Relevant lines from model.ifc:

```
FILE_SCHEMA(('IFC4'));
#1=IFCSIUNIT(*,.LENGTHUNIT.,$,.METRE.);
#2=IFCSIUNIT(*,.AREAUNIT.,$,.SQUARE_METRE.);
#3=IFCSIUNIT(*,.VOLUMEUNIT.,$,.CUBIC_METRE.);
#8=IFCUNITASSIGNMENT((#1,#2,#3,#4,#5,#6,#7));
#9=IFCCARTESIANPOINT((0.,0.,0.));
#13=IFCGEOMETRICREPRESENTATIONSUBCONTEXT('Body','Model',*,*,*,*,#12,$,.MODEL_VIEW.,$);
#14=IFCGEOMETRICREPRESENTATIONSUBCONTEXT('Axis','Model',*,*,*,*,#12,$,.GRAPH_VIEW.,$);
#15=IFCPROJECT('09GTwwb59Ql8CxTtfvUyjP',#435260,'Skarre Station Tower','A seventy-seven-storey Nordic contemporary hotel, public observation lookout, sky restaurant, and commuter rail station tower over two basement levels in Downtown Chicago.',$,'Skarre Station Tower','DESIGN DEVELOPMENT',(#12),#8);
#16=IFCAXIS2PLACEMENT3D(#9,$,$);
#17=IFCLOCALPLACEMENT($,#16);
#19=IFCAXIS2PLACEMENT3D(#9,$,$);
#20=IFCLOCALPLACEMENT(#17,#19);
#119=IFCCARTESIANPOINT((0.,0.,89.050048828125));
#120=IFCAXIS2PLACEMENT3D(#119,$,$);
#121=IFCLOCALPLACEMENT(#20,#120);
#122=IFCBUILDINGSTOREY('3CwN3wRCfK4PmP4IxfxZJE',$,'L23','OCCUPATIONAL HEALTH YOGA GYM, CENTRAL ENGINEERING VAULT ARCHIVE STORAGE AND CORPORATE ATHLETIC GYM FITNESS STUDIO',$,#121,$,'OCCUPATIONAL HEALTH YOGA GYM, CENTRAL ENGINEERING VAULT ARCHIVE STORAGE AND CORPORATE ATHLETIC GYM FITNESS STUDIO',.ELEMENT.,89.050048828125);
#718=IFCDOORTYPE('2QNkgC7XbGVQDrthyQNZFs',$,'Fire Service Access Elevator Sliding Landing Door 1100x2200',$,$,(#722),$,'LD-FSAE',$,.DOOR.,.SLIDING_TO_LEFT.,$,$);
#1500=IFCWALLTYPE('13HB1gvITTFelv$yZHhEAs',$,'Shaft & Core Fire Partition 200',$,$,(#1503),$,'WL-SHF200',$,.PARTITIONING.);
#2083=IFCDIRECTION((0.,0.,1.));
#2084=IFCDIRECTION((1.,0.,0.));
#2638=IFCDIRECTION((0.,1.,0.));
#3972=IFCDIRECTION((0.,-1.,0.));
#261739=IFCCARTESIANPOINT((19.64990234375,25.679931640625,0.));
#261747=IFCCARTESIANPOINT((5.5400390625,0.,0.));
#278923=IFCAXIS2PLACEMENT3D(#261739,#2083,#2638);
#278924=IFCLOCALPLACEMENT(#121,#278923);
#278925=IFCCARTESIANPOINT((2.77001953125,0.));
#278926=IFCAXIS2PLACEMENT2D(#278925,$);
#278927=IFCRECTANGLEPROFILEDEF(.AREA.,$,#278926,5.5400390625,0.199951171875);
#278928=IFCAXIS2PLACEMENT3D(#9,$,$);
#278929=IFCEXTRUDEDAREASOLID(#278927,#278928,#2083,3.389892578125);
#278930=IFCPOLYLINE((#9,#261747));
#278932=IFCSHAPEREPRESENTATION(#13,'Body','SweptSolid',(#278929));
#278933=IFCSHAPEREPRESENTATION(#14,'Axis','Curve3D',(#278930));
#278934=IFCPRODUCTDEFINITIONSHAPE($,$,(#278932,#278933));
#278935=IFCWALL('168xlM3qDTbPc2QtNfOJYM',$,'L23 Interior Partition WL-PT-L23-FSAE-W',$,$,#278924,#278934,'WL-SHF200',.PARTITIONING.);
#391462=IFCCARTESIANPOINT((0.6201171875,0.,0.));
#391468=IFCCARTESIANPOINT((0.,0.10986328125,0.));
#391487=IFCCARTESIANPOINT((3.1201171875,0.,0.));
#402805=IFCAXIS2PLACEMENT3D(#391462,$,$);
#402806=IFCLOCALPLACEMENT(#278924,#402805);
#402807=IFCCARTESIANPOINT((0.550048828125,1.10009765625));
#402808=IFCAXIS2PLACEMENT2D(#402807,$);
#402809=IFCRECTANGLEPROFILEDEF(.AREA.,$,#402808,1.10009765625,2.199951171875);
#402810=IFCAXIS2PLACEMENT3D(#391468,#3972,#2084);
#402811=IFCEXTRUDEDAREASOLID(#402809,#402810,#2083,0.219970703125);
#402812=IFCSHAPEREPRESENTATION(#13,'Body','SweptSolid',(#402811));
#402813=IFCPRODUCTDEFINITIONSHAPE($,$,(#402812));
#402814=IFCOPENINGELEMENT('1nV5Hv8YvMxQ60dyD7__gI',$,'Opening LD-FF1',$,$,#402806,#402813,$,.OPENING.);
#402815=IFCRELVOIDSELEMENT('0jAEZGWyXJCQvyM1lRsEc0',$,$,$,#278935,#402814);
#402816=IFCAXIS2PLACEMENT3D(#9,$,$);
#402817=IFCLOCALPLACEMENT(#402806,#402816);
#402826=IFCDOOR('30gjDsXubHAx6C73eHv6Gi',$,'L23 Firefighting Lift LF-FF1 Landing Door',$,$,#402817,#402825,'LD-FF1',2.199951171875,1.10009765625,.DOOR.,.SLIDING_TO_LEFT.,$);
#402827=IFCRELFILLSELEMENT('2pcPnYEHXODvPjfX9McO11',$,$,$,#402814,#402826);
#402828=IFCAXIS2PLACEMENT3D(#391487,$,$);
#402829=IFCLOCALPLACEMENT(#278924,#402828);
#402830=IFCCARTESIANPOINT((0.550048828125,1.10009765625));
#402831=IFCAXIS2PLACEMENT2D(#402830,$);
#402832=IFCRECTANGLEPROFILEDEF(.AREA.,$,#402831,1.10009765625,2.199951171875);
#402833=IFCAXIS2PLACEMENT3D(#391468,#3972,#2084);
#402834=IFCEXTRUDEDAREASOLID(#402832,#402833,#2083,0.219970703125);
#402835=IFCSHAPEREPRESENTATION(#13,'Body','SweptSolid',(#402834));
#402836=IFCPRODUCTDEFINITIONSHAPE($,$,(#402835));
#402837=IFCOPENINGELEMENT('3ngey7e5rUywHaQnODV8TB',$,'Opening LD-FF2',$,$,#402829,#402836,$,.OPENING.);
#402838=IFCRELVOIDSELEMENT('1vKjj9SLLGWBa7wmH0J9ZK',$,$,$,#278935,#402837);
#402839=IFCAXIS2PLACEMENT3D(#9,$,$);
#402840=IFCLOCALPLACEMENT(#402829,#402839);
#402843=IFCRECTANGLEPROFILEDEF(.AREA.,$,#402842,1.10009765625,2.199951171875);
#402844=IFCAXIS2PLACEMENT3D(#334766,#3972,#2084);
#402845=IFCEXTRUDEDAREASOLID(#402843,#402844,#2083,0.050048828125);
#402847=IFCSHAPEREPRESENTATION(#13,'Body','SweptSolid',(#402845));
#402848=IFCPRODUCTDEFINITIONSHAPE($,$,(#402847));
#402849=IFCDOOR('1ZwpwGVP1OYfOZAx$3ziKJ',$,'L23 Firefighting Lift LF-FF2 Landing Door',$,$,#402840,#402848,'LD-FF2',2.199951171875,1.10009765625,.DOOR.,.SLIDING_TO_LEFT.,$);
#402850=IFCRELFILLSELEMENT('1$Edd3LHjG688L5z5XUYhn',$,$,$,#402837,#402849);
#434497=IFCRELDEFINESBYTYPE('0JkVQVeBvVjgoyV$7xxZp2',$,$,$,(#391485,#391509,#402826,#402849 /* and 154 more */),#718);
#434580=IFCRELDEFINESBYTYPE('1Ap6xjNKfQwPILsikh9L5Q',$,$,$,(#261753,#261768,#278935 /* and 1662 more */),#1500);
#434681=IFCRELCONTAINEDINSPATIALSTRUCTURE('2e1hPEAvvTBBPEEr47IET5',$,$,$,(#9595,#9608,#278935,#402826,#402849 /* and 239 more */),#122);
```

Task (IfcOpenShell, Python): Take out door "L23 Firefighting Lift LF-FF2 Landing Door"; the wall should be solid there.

```python
import ifcopenshell
import ifcopenshell.api.feature
import ifcopenshell.api.root
import ifcopenshell.geom
import ifcopenshell.util.shape

model = ifcopenshell.open("model.ifc")
settings = ifcopenshell.geom.settings()


def volume(element):
    """Net volume in cubic metres, openings subtracted."""
    shape = ifcopenshell.geom.create_shape(settings, element)
    return ifcopenshell.util.shape.get_volume(shape.geometry)


door = model.by_id(402849)
opening = door.FillsVoids[0].RelatingOpeningElement
wall = opening.VoidsElements[0].RelatingBuildingElement
before = volume(wall)

ifcopenshell.api.root.remove_product(model, product=door)
ifcopenshell.api.feature.remove_feature(model, feature=opening)

after = volume(wall)

print(f"wall volume {before:.3f} -> {after:.3f} m3")

model.write("model_rev.ifc")
```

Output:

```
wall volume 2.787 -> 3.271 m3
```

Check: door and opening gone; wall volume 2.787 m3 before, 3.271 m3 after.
